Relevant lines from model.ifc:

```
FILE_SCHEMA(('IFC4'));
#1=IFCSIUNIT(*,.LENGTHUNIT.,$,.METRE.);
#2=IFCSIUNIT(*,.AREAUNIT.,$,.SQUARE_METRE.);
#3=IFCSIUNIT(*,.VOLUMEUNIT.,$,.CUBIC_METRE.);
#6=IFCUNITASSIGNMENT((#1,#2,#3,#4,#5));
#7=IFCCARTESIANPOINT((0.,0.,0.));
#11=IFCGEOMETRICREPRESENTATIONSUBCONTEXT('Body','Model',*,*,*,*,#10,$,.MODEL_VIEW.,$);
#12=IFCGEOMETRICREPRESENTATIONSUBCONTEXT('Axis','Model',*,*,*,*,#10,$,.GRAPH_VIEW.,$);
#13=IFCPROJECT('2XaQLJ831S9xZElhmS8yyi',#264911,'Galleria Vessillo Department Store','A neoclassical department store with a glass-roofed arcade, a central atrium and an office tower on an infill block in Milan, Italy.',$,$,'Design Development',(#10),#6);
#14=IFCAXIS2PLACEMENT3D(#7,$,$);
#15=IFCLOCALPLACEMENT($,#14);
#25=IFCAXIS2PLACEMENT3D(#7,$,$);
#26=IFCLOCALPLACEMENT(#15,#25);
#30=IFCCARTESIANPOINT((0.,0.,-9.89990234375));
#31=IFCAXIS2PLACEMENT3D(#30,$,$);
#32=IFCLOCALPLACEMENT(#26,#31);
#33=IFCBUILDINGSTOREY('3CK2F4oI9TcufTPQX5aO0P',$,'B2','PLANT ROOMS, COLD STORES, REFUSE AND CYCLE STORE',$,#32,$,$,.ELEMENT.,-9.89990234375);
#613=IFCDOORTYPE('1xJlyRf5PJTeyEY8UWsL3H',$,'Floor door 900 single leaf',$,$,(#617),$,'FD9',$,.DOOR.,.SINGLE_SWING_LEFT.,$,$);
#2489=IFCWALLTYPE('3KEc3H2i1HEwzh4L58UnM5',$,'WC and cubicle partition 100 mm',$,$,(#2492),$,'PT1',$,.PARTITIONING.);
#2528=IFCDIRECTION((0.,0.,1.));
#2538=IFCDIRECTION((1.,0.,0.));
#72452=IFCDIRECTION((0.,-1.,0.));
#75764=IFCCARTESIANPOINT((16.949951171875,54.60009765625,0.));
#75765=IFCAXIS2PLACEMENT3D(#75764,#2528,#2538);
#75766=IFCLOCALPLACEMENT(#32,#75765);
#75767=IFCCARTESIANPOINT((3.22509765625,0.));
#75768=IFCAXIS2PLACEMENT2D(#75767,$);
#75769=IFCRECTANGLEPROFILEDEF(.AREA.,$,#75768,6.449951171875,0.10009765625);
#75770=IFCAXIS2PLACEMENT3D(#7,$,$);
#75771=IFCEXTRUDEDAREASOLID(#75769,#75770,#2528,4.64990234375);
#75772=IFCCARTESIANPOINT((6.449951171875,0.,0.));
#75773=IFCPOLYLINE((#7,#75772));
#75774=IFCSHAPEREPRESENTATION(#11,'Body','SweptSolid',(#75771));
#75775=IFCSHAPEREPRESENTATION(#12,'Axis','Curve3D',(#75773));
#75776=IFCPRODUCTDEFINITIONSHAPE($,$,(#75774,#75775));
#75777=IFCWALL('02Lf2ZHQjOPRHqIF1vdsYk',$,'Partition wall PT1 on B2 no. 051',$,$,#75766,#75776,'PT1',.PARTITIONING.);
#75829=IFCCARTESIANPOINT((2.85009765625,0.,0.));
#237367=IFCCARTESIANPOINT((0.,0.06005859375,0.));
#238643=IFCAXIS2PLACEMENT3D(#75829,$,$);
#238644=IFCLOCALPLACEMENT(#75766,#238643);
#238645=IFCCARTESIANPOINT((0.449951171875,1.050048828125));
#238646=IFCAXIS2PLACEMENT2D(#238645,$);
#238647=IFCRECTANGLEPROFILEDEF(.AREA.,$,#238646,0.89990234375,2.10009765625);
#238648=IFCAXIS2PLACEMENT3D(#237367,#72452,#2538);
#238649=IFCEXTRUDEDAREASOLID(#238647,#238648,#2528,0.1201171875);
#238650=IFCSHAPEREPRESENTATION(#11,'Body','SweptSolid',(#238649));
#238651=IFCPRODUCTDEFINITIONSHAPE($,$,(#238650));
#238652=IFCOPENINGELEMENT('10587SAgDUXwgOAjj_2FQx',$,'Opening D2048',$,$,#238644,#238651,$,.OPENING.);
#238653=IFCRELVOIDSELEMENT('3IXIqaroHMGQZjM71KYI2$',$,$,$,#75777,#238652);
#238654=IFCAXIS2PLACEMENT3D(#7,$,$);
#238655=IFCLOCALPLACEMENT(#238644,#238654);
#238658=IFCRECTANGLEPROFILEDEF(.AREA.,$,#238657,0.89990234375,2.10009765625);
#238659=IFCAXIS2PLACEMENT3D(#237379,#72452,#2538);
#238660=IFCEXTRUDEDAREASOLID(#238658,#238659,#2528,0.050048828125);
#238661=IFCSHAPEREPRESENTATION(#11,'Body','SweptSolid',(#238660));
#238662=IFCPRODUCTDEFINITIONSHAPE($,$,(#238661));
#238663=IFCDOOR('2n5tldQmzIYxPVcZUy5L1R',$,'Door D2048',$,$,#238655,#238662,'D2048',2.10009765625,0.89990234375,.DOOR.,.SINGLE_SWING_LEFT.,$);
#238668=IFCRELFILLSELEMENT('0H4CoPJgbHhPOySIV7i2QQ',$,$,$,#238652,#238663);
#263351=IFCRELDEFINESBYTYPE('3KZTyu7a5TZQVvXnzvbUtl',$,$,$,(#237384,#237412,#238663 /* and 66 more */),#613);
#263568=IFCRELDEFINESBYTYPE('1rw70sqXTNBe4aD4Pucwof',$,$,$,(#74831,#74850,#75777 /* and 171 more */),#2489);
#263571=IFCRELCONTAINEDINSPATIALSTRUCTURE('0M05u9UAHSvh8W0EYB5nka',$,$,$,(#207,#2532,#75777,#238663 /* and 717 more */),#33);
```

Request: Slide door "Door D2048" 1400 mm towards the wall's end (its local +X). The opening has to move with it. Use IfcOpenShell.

```python
import ifcopenshell
import ifcopenshell.api.geometry
import ifcopenshell.util.placement
import ifcopenshell.util.unit

model = ifcopenshell.open("model.ifc")
unit_scale = ifcopenshell.util.unit.calculate_unit_scale(model)

door = model.by_guid("2n5tldQmzIYxPVcZUy5L1R")
opening = door.FillsVoids[0].RelatingOpeningElement
wall = opening.VoidsElements[0].RelatingBuildingElement

wall_matrix = ifcopenshell.util.placement.get_local_placement(wall.ObjectPlacement)
shift = wall_matrix[:3, 0] * 1.4 / unit_scale
before = ifcopenshell.util.placement.get_local_placement(door.ObjectPlacement)[:3, 3].copy()

# The door is placed relative to its opening, so it follows when the opening moves.
matrix = ifcopenshell.util.placement.get_local_placement(opening.ObjectPlacement)
matrix[:3, 3] += shift
ifcopenshell.api.geometry.edit_object_placement(
    model, product=opening, matrix=matrix, is_si=False, should_transform_children=True
)

after = ifcopenshell.util.placement.get_local_placement(door.ObjectPlacement)[:3, 3]
print("door moved by", (after - before).round(3) + 0.0)

model.write("model_v2.ifc")
```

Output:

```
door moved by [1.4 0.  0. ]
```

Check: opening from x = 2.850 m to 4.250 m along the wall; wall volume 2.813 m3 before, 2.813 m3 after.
